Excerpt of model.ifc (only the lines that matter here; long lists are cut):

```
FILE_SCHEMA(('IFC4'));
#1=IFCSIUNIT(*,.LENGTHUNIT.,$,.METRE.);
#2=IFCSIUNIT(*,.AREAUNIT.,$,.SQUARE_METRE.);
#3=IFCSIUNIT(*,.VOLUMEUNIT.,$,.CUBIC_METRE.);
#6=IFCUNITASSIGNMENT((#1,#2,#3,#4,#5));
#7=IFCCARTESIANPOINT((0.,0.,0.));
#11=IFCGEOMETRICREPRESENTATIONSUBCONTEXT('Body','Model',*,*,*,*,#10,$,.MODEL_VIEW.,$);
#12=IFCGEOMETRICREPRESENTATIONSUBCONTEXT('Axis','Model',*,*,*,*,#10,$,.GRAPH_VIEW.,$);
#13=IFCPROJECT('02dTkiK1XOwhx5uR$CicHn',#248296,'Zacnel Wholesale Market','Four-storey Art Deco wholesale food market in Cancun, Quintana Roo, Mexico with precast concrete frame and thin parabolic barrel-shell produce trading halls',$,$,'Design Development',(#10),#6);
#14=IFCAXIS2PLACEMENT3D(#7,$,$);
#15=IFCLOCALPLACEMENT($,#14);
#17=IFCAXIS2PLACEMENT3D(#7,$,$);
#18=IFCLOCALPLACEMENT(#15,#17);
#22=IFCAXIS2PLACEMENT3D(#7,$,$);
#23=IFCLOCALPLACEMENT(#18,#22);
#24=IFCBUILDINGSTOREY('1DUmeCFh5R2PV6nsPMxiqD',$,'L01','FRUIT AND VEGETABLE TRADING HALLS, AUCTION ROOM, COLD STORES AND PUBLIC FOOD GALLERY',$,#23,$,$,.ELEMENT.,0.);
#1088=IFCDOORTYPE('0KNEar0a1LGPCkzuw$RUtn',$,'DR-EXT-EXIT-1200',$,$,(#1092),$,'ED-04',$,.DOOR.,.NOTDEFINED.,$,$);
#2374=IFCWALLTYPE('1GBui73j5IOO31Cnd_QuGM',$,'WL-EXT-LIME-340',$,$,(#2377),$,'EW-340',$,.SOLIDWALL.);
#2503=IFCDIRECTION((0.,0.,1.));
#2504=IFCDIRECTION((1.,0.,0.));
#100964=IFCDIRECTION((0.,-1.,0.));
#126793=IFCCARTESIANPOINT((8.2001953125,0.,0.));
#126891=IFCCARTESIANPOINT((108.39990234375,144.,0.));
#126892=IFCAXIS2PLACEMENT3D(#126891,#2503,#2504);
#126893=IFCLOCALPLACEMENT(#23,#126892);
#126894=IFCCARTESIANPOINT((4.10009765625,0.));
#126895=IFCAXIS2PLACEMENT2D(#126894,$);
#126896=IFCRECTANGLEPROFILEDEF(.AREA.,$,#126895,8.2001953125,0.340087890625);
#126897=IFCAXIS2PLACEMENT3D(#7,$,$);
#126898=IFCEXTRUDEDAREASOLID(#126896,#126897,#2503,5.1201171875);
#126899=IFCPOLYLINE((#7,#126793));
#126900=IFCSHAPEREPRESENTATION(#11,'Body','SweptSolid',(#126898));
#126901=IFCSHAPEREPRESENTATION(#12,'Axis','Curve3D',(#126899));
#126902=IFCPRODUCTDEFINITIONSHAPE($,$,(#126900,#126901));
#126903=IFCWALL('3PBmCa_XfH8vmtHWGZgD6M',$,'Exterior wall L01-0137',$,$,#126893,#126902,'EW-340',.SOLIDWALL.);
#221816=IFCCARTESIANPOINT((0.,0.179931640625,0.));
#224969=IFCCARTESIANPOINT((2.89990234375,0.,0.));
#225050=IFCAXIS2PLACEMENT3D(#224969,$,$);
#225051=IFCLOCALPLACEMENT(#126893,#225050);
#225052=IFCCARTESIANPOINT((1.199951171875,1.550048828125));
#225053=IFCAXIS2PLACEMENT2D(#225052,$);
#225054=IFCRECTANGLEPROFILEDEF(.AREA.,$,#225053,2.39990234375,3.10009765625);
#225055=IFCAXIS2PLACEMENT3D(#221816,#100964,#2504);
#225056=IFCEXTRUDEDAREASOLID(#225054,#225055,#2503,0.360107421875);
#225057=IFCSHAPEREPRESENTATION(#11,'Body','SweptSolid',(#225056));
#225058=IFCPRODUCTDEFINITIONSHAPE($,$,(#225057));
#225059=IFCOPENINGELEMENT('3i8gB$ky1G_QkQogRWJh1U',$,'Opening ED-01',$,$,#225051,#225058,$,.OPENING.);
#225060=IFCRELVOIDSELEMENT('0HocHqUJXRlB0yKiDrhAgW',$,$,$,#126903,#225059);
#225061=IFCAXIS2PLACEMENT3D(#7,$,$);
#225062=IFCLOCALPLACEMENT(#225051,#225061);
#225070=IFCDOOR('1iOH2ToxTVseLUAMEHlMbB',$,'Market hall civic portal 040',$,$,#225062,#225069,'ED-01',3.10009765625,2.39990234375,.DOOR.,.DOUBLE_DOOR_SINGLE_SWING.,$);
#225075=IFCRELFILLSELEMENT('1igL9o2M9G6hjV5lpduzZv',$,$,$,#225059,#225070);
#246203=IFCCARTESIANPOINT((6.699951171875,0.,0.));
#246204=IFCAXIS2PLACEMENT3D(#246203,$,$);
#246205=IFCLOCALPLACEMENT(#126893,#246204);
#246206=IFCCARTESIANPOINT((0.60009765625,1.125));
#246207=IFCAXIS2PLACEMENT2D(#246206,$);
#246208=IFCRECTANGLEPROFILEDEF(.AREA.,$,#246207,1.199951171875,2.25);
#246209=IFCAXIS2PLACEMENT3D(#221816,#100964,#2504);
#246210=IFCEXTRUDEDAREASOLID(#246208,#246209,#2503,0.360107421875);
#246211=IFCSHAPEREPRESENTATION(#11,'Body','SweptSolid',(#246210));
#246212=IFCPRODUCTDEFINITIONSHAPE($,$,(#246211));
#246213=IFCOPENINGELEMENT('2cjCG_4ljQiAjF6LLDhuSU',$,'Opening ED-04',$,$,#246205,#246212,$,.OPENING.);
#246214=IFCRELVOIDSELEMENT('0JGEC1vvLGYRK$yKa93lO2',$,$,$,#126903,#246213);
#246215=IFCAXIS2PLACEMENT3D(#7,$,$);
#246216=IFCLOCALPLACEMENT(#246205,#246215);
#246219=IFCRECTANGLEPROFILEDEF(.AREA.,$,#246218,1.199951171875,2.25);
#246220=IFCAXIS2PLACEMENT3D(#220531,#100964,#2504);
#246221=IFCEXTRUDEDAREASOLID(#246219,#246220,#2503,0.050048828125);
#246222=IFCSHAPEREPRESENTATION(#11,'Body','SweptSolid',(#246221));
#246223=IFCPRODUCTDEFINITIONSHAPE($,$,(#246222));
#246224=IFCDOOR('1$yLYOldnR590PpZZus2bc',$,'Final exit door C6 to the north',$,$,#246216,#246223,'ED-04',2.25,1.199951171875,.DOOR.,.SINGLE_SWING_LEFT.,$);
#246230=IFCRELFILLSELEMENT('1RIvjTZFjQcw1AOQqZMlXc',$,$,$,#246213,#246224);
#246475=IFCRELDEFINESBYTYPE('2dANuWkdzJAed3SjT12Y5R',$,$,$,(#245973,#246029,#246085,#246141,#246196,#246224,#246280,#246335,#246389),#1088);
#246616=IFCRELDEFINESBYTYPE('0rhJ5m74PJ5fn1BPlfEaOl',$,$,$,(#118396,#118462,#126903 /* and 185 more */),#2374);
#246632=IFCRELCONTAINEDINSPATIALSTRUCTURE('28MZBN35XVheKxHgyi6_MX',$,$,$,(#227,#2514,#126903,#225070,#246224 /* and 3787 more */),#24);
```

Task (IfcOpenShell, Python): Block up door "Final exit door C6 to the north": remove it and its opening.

```python
import ifcopenshell
import ifcopenshell.api.feature
import ifcopenshell.api.root
import ifcopenshell.geom
import ifcopenshell.util.shape

model = ifcopenshell.open("model.ifc")
settings = ifcopenshell.geom.settings()


def volume(element):
    """Net volume in cubic metres, openings subtracted."""
    shape = ifcopenshell.geom.create_shape(settings, element)
    return ifcopenshell.util.shape.get_volume(shape.geometry)


door = model.by_id(246224)
opening = door.FillsVoids[0].RelatingOpeningElement
wall = opening.VoidsElements[0].RelatingBuildingElement
before = volume(wall)

ifcopenshell.api.root.remove_product(model, product=door)
ifcopenshell.api.feature.remove_feature(model, feature=opening)

after = volume(wall)

print(f"wall volume {before:.3f} -> {after:.3f} m3")

model.write("model_v2.ifc")
```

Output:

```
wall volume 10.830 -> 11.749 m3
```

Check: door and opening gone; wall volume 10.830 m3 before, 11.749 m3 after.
